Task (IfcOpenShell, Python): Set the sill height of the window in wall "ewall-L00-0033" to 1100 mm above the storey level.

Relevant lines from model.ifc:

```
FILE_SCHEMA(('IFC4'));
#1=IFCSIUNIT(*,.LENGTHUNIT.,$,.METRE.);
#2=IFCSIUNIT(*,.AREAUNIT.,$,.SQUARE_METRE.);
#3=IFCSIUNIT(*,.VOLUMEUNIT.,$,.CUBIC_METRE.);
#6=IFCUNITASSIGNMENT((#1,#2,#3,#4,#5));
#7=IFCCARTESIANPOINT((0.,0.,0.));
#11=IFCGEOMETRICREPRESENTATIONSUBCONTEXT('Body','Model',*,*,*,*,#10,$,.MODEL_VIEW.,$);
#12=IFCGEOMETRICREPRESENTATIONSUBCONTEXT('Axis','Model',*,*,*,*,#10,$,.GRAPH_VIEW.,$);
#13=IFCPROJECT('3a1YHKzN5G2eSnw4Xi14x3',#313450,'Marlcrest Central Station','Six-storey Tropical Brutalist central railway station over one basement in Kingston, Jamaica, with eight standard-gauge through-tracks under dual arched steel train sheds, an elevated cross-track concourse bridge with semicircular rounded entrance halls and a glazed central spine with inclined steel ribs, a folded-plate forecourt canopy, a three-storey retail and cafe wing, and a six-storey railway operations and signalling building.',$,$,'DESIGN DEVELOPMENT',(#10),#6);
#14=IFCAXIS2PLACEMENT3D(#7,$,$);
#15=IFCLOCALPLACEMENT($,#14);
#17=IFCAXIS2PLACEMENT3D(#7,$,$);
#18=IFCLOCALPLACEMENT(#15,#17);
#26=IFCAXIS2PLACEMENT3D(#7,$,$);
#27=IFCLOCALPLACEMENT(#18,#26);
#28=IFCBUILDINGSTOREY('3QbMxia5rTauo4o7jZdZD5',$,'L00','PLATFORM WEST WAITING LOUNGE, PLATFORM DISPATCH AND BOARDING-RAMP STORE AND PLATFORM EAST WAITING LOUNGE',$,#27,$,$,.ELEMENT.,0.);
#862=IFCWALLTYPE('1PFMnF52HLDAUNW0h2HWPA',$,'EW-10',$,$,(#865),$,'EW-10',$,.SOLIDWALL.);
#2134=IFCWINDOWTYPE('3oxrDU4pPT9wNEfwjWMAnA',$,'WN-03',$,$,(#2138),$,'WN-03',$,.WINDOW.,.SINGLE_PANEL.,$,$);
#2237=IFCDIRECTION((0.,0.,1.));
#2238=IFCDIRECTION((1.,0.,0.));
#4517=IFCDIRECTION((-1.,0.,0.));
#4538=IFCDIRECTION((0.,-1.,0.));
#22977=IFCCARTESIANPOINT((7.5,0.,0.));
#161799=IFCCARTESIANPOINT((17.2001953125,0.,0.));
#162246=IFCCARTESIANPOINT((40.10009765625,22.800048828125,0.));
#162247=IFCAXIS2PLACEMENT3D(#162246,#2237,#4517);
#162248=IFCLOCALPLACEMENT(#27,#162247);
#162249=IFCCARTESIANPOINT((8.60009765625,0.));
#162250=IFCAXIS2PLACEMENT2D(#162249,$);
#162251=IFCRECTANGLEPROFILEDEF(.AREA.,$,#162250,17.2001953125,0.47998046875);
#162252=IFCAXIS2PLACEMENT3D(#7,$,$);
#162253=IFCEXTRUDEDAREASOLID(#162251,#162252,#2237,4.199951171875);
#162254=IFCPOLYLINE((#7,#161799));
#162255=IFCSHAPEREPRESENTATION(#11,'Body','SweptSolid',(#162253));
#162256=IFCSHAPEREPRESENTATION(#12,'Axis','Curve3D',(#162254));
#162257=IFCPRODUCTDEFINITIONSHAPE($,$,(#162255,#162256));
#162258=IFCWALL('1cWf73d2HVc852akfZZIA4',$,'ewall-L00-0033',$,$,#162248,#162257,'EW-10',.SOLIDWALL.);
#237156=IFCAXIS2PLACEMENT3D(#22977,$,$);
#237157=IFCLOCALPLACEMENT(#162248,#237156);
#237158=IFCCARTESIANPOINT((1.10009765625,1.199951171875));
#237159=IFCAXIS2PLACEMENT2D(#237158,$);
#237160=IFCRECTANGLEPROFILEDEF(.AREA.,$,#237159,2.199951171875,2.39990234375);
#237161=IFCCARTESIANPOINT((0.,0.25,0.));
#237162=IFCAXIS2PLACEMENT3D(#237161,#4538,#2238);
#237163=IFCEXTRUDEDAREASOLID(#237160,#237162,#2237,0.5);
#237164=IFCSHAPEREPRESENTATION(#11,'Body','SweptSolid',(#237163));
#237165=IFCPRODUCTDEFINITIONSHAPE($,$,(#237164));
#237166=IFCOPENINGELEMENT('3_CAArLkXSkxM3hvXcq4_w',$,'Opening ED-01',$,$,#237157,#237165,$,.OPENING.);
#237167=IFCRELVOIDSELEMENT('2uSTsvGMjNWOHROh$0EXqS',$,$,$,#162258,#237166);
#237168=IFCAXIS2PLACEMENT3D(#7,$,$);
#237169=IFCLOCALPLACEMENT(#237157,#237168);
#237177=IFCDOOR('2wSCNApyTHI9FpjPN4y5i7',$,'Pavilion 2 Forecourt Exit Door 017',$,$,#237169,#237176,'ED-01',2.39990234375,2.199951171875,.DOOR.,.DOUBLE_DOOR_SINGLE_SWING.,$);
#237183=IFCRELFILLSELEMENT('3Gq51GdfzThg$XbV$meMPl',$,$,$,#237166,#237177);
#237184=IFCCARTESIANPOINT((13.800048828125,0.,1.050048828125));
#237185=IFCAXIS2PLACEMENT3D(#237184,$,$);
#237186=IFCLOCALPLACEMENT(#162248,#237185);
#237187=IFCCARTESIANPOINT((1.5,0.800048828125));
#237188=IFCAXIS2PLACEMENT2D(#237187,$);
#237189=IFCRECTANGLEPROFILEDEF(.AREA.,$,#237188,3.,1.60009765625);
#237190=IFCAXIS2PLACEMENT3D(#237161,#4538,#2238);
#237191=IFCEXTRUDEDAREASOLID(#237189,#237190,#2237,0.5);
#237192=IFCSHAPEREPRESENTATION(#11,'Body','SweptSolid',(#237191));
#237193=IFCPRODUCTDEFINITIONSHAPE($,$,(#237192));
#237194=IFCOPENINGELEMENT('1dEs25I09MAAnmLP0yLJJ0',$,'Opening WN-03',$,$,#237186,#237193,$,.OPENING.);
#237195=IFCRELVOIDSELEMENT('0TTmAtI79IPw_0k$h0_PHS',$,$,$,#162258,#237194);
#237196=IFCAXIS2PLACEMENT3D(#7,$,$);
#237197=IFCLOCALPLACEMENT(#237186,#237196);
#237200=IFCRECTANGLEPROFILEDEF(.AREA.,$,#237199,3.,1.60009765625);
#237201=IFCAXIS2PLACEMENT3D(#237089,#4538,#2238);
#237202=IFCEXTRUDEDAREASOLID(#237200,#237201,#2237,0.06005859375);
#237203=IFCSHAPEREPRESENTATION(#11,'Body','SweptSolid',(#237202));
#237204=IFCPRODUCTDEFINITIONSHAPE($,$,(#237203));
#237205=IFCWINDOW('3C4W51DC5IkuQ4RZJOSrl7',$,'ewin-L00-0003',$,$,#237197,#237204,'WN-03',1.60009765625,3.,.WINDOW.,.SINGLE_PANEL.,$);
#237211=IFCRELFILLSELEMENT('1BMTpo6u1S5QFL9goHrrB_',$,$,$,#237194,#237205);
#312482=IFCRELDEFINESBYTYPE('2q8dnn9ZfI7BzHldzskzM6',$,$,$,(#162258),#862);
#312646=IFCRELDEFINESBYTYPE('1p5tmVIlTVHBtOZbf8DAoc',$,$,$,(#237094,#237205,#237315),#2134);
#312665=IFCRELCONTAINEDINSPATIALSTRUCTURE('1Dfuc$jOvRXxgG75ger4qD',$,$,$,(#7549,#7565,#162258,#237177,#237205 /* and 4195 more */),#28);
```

```python
import numpy as np
import ifcopenshell
import ifcopenshell.api.geometry
import ifcopenshell.geom
import ifcopenshell.util.element
import ifcopenshell.util.placement
import ifcopenshell.util.shape
import ifcopenshell.util.unit

model = ifcopenshell.open("model.ifc")
unit_scale = ifcopenshell.util.unit.calculate_unit_scale(model)

window = model.by_guid("3C4W51DC5IkuQ4RZJOSrl7")
opening = window.FillsVoids[0].RelatingOpeningElement
storey = ifcopenshell.util.element.get_container(window, ifc_class="IfcBuildingStorey")
level = ifcopenshell.util.placement.get_local_placement(storey.ObjectPlacement)[2, 3]

# The opening's origin need not be at the sill, so measure its lowest point.
shape = ifcopenshell.geom.create_shape(ifcopenshell.geom.settings(), opening)
bottom = ifcopenshell.util.shape.get_shape_bottom_elevation(shape, shape.geometry) / unit_scale
dz = level + 1.1 / unit_scale - bottom

shift = np.array([0.0, 0.0, dz])
# The window is placed relative to its opening, so it follows when the opening moves.
matrix = ifcopenshell.util.placement.get_local_placement(opening.ObjectPlacement)
matrix[:3, 3] += shift
ifcopenshell.api.geometry.edit_object_placement(
    model, product=opening, matrix=matrix, is_si=False, should_transform_children=True
)

print(f"moved by {dz * unit_scale:+.3f} m")

model.write("model_updated.ifc")
```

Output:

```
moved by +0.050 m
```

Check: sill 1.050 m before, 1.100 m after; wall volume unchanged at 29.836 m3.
